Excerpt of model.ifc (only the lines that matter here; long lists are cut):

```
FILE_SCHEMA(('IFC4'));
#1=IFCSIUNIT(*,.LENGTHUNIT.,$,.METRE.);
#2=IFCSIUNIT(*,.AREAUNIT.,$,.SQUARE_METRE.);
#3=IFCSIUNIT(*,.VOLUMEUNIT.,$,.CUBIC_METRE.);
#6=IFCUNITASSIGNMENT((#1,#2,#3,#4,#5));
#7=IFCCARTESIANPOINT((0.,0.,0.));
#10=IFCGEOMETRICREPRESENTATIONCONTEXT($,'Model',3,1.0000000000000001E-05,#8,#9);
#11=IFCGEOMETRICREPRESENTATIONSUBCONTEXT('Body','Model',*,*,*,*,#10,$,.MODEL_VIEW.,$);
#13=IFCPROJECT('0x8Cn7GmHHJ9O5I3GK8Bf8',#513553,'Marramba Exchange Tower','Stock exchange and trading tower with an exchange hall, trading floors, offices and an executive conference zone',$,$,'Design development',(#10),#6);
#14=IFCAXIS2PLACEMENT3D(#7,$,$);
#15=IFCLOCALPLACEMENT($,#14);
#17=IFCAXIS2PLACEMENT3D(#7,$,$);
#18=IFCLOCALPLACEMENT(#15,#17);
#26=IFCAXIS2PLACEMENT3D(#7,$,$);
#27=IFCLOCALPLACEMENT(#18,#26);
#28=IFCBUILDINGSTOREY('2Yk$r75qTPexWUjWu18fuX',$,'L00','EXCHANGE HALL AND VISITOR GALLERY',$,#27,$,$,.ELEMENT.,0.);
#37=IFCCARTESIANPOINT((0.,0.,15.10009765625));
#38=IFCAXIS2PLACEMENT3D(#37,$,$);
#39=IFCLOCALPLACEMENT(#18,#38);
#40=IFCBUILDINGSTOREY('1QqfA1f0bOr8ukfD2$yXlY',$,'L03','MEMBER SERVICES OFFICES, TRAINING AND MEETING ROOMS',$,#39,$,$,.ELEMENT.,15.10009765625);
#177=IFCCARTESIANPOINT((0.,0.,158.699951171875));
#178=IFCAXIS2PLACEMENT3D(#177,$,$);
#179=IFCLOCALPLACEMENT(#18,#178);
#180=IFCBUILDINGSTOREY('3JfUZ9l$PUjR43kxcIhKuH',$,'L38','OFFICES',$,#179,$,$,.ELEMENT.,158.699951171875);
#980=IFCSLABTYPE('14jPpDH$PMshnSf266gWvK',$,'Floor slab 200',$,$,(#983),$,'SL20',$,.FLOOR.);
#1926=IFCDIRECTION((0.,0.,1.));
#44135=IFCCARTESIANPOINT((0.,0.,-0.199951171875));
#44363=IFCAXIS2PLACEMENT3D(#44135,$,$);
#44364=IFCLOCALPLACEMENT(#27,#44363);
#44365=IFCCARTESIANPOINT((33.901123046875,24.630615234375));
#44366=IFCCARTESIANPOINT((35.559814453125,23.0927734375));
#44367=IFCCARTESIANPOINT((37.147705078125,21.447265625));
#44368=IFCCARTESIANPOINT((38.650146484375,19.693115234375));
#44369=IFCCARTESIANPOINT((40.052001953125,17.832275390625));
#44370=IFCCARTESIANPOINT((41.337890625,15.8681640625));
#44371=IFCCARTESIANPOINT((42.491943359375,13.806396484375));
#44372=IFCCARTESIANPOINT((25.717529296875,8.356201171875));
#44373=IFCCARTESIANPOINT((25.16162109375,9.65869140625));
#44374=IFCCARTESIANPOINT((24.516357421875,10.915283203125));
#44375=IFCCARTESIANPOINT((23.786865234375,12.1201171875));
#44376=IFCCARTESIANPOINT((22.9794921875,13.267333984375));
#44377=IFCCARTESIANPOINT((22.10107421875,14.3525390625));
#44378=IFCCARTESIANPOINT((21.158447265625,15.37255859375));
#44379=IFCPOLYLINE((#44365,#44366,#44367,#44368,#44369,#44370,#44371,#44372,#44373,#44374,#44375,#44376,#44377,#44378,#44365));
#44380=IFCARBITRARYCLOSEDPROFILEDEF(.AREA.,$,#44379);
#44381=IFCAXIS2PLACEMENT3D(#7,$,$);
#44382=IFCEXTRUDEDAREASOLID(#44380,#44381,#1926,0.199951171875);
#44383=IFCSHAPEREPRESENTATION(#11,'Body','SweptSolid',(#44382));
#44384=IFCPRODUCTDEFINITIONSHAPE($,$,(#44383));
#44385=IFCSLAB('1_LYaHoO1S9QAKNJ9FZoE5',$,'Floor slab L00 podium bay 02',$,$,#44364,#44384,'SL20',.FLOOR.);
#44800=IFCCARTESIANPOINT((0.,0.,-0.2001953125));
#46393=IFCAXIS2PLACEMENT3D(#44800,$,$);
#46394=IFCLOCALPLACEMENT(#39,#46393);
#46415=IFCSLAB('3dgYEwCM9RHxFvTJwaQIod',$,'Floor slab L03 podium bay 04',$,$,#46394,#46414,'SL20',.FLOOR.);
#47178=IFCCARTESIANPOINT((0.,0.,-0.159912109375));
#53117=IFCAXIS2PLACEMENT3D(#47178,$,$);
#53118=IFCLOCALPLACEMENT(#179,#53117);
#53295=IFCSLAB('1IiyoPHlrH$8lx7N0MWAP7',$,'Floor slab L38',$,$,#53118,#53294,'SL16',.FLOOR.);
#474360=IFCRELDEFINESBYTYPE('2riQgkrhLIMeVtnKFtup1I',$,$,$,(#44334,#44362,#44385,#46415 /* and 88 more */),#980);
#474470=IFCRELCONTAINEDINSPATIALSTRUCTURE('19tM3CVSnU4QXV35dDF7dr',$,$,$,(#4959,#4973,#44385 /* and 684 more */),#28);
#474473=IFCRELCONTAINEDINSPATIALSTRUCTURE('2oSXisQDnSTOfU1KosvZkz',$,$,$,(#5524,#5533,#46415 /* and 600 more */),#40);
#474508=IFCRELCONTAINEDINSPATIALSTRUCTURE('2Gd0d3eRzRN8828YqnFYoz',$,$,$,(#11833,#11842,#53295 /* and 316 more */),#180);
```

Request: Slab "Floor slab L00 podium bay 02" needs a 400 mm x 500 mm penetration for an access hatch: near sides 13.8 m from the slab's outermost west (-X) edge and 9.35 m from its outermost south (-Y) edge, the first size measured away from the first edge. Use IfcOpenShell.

```python
import numpy as np
import ifcopenshell
import ifcopenshell.api.feature
import ifcopenshell.api.geometry
import ifcopenshell.api.root
import ifcopenshell.geom
import ifcopenshell.util.placement
import ifcopenshell.util.representation
import ifcopenshell.util.shape
import ifcopenshell.util.unit

model = ifcopenshell.open("model.ifc")
unit_scale = ifcopenshell.util.unit.calculate_unit_scale(model)
settings = ifcopenshell.geom.settings()


def volume(element):
    """Net volume in cubic metres, openings subtracted."""
    shape = ifcopenshell.geom.create_shape(settings, element)
    return ifcopenshell.util.shape.get_volume(shape.geometry)


slab = model.by_guid("1_LYaHoO1S9QAKNJ9FZoE5")
before = volume(slab)

# Extent in the slab's own axes, in metres. The edges named are its -X and -Y sides.
slab_shape = ifcopenshell.geom.create_shape(settings, slab)
vertices = ifcopenshell.util.shape.get_vertices(slab_shape.geometry)
x_min, y_min, bottom = vertices.min(axis=0)
top = vertices[:, 2].max()

opening = ifcopenshell.api.root.create_entity(model, ifc_class="IfcOpeningElement", name="Access hatch opening", predefined_type="OPENING")
context = ifcopenshell.util.representation.get_context(model, "Model", "Body", "MODEL_VIEW")
width, depth = 0.4, 0.5
outline = [(0.0, 0.0), (width, 0.0), (width, depth), (0.0, depth), (0.0, 0.0)]
# Overshoot both faces by 50 mm so the cut is clean.
shape = ifcopenshell.api.geometry.add_slab_representation(
    model, context=context, depth=top - bottom + 0.1, polyline=outline
)
ifcopenshell.api.geometry.assign_representation(model, product=opening, representation=shape)

matrix = ifcopenshell.util.placement.get_local_placement(slab.ObjectPlacement)
matrix[:, 3] = matrix @ np.append(np.array([x_min + 13.8, y_min + 9.35, bottom - 0.05]) / unit_scale, 1.0)
ifcopenshell.api.geometry.edit_object_placement(model, product=opening, matrix=matrix, is_si=False)
ifcopenshell.api.feature.add_feature(model, feature=opening, element=slab)

after = volume(slab)

print(f"slab volume {before:.3f} -> {after:.3f} m3")

model.write("model-out.ifc")
```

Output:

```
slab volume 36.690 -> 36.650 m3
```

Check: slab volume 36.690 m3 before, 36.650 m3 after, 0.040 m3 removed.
